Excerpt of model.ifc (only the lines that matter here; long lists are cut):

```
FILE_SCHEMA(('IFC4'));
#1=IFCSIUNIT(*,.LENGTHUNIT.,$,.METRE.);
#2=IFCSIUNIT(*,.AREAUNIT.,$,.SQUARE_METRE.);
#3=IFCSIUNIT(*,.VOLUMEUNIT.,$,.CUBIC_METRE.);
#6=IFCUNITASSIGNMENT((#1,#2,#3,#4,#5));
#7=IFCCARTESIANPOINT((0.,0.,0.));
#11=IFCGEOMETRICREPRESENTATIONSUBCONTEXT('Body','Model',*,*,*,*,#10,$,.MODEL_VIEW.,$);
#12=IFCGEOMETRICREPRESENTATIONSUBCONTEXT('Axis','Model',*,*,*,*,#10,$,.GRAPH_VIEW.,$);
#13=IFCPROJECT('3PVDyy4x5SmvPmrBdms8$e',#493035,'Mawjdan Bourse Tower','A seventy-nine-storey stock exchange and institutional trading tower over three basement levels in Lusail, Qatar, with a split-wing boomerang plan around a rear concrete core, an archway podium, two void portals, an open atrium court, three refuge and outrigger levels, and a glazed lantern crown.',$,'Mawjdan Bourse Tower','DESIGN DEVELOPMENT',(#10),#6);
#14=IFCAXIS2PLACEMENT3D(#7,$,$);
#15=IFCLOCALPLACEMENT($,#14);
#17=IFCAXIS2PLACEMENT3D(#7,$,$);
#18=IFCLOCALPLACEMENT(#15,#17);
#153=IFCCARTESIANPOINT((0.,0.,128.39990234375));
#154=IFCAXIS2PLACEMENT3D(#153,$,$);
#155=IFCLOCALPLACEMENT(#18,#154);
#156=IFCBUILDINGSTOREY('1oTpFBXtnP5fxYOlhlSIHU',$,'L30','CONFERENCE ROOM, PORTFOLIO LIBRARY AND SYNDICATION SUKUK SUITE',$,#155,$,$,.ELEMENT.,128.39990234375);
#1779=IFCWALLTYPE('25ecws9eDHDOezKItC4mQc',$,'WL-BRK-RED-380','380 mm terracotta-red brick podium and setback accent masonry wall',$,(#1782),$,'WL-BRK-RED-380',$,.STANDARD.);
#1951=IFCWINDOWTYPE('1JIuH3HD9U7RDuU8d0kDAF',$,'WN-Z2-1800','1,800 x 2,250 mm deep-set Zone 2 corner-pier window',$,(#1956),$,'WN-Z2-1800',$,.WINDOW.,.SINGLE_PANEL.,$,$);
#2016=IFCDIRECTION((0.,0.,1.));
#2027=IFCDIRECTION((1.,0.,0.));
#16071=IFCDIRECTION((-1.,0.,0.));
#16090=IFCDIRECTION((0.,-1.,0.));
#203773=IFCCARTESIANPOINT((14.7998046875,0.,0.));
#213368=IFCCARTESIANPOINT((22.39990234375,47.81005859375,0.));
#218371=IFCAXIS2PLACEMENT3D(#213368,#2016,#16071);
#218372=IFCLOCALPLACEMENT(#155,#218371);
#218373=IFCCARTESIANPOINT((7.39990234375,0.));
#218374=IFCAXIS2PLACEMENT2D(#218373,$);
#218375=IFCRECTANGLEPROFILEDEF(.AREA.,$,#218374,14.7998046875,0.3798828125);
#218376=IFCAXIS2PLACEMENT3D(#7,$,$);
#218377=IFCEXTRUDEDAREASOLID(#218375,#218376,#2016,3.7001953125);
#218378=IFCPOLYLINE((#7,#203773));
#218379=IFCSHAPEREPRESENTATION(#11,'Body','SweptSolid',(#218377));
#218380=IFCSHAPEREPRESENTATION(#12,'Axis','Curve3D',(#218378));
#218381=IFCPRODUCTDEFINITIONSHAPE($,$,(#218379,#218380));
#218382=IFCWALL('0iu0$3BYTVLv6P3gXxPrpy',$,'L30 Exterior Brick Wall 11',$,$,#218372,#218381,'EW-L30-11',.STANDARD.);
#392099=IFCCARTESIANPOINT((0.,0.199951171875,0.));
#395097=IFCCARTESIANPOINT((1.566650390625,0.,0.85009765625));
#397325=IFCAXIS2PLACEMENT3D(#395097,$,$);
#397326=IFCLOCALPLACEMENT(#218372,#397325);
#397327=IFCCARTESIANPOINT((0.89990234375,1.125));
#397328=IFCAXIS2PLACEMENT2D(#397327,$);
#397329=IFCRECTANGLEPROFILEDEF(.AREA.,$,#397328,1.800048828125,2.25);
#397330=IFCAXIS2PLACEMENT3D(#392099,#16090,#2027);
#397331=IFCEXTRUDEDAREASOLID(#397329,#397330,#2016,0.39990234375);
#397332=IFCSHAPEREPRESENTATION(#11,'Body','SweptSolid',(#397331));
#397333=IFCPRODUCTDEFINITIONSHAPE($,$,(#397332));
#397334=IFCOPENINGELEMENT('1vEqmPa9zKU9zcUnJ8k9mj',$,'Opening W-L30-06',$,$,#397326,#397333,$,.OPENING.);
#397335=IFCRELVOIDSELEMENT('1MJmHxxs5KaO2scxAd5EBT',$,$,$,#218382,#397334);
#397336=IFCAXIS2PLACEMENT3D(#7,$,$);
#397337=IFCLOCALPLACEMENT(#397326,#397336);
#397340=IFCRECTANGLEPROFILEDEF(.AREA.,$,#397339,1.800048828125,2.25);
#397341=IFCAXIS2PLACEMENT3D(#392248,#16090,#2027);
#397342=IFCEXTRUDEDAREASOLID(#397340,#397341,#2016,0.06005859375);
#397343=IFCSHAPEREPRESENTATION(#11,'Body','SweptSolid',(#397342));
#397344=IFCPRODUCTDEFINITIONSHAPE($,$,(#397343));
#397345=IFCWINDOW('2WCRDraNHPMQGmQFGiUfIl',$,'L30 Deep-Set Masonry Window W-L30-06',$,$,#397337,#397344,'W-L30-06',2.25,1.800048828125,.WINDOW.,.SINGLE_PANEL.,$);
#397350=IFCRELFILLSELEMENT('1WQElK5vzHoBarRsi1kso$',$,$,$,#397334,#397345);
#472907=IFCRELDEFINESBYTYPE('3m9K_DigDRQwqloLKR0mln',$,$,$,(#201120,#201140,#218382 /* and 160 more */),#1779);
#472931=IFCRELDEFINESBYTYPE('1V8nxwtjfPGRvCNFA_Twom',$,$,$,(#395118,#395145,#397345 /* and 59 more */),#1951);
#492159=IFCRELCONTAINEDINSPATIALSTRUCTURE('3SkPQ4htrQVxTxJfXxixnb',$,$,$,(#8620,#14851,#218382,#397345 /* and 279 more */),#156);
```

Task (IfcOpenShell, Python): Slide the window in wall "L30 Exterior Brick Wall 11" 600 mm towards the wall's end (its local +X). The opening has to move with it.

```python
import ifcopenshell
import ifcopenshell.api.geometry
import ifcopenshell.util.placement

model = ifcopenshell.open("model.ifc")

window = model.by_id(397345)
opening = window.FillsVoids[0].RelatingOpeningElement
wall = opening.VoidsElements[0].RelatingBuildingElement

wall_matrix = ifcopenshell.util.placement.get_local_placement(wall.ObjectPlacement)
shift = wall_matrix[:3, 0] * 0.6
before = ifcopenshell.util.placement.get_local_placement(window.ObjectPlacement)[:3, 3].copy()

# The window is placed relative to its opening, so it follows when the opening moves.
matrix = ifcopenshell.util.placement.get_local_placement(opening.ObjectPlacement)
matrix[:3, 3] += shift
ifcopenshell.api.geometry.edit_object_placement(
    model, product=opening, matrix=matrix, is_si=False, should_transform_children=True
)

after = ifcopenshell.util.placement.get_local_placement(window.ObjectPlacement)[:3, 3]
print("window moved by", (after - before).round(3) + 0.0)

model.write("model_edited.ifc")
```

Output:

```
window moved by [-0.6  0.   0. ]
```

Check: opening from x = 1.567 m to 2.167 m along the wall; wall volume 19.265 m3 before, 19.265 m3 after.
